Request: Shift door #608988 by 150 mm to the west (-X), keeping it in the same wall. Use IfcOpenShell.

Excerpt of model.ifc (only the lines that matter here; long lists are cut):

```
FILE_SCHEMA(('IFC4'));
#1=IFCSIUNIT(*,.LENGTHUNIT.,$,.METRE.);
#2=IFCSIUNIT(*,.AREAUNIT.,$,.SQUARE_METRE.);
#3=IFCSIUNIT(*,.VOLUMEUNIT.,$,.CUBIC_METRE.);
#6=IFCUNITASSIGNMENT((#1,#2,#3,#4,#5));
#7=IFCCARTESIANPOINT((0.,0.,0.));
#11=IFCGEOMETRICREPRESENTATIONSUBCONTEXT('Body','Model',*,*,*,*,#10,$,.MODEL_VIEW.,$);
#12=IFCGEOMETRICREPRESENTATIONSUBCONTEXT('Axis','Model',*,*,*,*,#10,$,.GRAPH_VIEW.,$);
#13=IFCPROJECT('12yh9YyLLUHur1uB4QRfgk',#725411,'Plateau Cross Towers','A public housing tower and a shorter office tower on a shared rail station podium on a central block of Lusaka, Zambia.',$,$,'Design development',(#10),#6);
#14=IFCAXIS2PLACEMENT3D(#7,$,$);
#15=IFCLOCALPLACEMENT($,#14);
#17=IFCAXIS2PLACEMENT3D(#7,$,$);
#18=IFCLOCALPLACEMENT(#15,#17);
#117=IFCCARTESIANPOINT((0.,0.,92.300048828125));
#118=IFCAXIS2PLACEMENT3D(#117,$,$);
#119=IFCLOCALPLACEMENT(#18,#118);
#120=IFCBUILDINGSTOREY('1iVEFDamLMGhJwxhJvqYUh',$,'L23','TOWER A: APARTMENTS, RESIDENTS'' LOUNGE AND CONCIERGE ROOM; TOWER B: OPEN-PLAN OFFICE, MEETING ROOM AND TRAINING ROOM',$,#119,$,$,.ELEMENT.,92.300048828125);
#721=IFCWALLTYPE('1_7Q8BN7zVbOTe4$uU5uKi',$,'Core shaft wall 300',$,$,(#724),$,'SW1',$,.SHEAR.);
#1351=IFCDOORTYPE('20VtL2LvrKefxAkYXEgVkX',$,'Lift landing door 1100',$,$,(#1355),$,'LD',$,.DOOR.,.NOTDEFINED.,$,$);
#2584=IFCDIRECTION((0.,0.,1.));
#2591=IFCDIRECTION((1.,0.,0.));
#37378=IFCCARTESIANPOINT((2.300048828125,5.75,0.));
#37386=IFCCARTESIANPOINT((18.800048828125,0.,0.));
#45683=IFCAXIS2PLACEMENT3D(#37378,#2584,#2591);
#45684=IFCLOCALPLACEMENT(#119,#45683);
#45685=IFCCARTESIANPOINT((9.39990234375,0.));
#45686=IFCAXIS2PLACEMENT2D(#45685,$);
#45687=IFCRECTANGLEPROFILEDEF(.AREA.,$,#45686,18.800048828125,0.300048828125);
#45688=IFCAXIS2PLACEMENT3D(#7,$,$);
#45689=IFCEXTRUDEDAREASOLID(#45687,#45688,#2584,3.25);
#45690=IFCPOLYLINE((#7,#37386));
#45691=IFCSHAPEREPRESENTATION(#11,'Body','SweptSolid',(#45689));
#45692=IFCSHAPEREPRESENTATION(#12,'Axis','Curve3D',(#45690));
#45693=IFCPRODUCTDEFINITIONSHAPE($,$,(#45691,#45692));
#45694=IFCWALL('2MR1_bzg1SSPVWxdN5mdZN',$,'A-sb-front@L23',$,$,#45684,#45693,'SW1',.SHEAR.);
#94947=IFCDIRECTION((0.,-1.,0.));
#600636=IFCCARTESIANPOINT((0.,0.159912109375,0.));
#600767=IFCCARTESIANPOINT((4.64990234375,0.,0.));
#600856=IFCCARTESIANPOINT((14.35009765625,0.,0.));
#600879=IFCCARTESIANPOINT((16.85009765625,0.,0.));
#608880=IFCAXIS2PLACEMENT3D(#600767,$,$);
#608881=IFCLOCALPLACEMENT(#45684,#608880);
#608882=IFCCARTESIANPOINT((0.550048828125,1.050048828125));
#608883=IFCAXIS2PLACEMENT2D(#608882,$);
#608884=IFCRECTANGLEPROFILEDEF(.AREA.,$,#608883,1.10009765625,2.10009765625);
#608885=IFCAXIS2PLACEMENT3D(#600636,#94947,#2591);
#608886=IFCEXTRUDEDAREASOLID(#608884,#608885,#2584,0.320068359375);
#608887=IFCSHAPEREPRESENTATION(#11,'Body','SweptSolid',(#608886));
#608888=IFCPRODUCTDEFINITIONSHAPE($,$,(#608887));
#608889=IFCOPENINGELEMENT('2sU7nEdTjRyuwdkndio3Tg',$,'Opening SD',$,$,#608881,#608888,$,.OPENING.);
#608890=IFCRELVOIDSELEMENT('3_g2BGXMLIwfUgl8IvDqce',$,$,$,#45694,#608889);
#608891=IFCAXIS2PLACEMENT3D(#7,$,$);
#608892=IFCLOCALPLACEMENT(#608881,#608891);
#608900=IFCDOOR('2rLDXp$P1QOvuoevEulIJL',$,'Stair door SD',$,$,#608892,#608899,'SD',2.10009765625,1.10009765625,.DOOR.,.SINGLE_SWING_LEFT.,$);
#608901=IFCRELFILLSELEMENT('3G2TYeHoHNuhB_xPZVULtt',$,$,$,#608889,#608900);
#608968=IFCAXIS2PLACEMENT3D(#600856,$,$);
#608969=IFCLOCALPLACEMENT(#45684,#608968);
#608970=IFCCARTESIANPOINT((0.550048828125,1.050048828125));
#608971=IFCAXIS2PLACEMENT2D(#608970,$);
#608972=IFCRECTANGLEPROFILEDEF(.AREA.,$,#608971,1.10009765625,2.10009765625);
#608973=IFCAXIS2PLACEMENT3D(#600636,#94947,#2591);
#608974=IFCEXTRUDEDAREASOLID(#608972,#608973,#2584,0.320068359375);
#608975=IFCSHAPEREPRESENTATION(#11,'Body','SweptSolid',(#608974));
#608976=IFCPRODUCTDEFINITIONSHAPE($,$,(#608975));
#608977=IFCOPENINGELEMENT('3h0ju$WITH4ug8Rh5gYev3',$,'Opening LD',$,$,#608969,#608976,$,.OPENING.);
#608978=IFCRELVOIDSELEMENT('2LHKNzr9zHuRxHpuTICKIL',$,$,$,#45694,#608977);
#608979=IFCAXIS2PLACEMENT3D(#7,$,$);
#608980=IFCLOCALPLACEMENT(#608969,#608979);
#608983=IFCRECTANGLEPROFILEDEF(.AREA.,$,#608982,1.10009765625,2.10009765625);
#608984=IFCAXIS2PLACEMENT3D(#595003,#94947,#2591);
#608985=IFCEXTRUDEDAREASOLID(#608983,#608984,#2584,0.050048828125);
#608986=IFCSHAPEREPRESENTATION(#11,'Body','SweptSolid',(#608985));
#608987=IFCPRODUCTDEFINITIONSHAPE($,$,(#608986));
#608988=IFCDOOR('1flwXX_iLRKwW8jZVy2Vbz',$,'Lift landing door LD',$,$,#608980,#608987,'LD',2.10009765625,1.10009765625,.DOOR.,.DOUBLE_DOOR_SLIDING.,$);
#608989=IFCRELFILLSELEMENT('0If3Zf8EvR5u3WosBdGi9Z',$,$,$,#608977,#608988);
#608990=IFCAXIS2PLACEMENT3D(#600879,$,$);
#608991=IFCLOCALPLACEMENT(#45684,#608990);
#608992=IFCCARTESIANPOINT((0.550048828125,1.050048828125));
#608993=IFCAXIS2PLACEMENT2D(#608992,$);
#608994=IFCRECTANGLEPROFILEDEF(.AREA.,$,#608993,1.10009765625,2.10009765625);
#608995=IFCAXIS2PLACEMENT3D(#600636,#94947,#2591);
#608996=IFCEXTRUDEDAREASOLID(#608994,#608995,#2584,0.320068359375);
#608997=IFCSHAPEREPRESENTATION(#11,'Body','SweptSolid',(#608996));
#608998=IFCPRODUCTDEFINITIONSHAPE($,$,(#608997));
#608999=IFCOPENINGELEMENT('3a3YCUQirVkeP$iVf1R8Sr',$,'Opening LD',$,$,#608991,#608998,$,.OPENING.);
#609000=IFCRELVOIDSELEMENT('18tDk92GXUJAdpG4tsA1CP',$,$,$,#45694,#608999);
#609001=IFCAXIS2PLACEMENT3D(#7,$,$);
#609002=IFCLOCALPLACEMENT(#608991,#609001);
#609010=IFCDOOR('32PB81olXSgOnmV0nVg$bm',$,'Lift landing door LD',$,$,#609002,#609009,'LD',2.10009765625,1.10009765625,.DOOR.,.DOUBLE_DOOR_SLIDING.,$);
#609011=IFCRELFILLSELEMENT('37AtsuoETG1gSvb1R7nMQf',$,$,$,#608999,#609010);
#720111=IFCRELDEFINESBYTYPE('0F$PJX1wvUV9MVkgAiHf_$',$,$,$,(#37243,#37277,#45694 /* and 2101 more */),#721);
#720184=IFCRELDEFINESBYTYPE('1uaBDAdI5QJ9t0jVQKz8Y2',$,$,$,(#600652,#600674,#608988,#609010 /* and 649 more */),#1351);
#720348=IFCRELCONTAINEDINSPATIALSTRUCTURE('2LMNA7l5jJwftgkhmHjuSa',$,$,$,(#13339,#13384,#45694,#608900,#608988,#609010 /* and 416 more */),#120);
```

```python
import ifcopenshell
import ifcopenshell.api.geometry
import ifcopenshell.util.placement

model = ifcopenshell.open("model.ifc")

door = model.by_id(608988)
opening = door.FillsVoids[0].RelatingOpeningElement
wall = opening.VoidsElements[0].RelatingBuildingElement

wall_matrix = ifcopenshell.util.placement.get_local_placement(wall.ObjectPlacement)
shift = wall_matrix[:3, 0] * -0.15
before = ifcopenshell.util.placement.get_local_placement(door.ObjectPlacement)[:3, 3].copy()

# The door is placed relative to its opening, so it follows when the opening moves.
matrix = ifcopenshell.util.placement.get_local_placement(opening.ObjectPlacement)
matrix[:3, 3] += shift
ifcopenshell.api.geometry.edit_object_placement(
    model, product=opening, matrix=matrix, is_si=False, should_transform_children=True
)

after = ifcopenshell.util.placement.get_local_placement(door.ObjectPlacement)[:3, 3]
print("door moved by", (after - before).round(3) + 0.0)

model.write("model_edited.ifc")
```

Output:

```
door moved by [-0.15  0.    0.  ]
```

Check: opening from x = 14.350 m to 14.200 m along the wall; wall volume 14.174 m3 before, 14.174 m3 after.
